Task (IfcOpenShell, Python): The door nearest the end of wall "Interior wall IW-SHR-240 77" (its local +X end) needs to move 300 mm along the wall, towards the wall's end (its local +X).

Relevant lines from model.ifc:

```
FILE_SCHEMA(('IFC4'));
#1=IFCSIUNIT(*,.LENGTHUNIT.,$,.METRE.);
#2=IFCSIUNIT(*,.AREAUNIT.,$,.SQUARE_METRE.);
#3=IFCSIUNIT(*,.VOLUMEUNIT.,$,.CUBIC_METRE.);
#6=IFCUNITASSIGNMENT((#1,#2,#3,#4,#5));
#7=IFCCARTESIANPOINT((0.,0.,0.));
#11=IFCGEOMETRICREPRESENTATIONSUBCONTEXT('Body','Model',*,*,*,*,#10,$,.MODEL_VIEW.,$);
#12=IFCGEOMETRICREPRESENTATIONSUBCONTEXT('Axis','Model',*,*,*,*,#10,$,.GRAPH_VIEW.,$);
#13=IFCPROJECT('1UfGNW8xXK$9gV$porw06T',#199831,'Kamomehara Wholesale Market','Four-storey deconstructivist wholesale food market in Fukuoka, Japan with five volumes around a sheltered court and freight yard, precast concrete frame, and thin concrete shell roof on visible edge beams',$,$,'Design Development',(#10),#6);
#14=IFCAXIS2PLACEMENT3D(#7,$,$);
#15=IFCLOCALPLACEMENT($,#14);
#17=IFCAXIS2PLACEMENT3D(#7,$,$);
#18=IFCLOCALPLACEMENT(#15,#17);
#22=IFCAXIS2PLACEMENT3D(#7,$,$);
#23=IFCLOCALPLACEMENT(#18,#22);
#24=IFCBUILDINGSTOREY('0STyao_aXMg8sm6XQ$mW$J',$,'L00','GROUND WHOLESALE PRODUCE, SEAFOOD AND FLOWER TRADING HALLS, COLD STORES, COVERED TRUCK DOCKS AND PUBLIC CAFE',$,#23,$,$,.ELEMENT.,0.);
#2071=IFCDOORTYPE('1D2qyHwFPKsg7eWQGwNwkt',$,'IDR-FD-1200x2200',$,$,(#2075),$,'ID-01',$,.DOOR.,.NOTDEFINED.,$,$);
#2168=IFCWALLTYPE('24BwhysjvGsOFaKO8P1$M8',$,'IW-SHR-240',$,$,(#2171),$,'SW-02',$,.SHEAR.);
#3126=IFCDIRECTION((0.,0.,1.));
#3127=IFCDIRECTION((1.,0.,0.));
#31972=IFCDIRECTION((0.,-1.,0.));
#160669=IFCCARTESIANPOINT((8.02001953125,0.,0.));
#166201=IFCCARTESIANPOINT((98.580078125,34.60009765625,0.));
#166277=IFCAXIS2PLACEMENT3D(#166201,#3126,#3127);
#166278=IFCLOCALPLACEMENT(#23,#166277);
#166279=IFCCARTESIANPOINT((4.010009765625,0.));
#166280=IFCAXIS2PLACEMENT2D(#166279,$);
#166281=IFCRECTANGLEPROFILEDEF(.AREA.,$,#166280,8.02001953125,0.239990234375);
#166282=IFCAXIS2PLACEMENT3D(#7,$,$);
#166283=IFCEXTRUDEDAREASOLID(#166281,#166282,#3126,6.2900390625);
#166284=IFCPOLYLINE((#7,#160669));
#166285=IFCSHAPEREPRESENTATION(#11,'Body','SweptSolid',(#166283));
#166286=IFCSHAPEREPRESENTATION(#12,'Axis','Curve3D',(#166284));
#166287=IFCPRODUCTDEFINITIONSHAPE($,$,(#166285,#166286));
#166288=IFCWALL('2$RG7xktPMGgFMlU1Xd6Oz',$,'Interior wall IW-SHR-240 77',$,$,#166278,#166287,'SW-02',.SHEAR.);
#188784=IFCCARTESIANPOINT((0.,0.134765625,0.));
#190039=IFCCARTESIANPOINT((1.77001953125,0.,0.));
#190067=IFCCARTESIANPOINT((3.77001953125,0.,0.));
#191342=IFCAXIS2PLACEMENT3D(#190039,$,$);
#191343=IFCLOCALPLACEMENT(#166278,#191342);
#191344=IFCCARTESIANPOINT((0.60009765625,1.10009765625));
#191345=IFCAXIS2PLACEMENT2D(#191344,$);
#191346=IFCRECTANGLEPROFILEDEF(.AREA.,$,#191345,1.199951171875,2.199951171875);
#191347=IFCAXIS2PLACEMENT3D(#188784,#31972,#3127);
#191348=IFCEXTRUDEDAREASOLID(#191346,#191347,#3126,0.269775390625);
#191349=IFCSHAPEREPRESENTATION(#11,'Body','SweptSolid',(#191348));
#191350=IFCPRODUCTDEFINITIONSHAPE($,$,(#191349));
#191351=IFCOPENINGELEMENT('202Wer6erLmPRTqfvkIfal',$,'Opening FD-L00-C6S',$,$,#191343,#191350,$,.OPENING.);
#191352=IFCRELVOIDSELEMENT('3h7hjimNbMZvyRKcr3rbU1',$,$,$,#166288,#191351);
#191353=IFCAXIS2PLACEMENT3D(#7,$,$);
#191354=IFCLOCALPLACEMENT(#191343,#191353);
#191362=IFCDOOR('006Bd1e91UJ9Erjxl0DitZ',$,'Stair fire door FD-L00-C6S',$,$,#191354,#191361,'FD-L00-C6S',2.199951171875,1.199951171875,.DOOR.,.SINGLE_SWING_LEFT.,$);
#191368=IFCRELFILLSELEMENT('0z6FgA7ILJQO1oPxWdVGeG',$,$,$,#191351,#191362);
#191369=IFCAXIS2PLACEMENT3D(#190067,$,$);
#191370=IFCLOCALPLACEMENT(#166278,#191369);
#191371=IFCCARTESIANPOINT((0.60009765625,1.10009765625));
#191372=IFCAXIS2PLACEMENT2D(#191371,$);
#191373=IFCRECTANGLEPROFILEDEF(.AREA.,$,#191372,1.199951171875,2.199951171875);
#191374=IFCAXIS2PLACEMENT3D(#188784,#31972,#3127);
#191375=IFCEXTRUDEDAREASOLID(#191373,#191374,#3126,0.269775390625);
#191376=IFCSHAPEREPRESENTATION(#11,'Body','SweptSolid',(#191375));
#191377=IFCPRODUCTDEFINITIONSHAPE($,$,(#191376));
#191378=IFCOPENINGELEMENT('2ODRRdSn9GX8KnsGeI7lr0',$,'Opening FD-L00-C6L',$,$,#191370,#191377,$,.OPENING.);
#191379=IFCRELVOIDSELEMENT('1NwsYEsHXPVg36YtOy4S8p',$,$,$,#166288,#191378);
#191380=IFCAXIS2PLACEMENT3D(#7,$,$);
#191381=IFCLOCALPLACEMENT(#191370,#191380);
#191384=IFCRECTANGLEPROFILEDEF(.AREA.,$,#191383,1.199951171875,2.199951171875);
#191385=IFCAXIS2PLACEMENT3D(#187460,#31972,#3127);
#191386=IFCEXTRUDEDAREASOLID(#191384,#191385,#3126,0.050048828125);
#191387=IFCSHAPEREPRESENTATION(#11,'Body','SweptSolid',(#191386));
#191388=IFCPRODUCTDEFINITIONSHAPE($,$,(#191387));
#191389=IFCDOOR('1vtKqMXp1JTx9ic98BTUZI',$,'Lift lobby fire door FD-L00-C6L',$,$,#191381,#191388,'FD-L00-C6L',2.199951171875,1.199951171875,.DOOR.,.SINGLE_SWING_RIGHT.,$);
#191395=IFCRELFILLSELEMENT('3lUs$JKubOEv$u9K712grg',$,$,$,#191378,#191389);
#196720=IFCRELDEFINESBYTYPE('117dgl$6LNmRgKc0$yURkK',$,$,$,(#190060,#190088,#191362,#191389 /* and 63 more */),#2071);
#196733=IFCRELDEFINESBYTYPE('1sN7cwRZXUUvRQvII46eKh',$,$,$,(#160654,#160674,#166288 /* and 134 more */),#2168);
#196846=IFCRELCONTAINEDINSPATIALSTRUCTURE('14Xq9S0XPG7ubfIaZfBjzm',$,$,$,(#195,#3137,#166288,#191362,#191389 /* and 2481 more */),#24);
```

```python
import ifcopenshell
import ifcopenshell.api.geometry
import ifcopenshell.util.placement
import ifcopenshell.util.unit

model = ifcopenshell.open("model.ifc")
unit_scale = ifcopenshell.util.unit.calculate_unit_scale(model)

door = model.by_guid("1vtKqMXp1JTx9ic98BTUZI")
opening = door.FillsVoids[0].RelatingOpeningElement
wall = opening.VoidsElements[0].RelatingBuildingElement

wall_matrix = ifcopenshell.util.placement.get_local_placement(wall.ObjectPlacement)
shift = wall_matrix[:3, 0] * 0.3 / unit_scale
before = ifcopenshell.util.placement.get_local_placement(door.ObjectPlacement)[:3, 3].copy()

# The door is placed relative to its opening, so it follows when the opening moves.
matrix = ifcopenshell.util.placement.get_local_placement(opening.ObjectPlacement)
matrix[:3, 3] += shift
ifcopenshell.api.geometry.edit_object_placement(
    model, product=opening, matrix=matrix, is_si=False, should_transform_children=True
)

after = ifcopenshell.util.placement.get_local_placement(door.ObjectPlacement)[:3, 3]
print("door moved by", (after - before).round(3) + 0.0)

model.write("model-out.ifc")
```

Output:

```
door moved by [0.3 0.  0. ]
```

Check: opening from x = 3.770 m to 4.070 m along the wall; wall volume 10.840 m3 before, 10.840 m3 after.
